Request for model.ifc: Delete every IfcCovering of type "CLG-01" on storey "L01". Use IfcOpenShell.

First a look at what the model holds.

```python
import ifcopenshell
import ifcopenshell.util.element

model = ifcopenshell.open("model.ifc")
print(model.schema)
storey = next(s for s in model.by_type("IfcBuildingStorey") if s.Name == "L01")
coverings = [e for e in ifcopenshell.util.element.get_decomposition(storey) if e.is_a("IfcCovering")]
seen = {}
for e in coverings:
    element_type = ifcopenshell.util.element.get_type(e)
    name = element_type.Name if element_type not in (None, e) else None
    seen[name] = seen.get(name, 0) + 1
for name, count in sorted(seen.items(), key=str):
    print(count, "x", name)
```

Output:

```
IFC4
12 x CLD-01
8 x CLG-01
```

```python
import ifcopenshell
import ifcopenshell.api.root
import ifcopenshell.util.element

model = ifcopenshell.open("model.ifc")

storey = next(s for s in model.by_type("IfcBuildingStorey") if s.Name == "L01")
coverings = [e for e in ifcopenshell.util.element.get_decomposition(storey) if e.is_a("IfcCovering")]
targets = [e for e in coverings if (t := ifcopenshell.util.element.get_type(e)) not in (None, e) and t.Name == "CLG-01"]

for e in targets:
    ifcopenshell.api.root.remove_product(model, product=e)
print(len(targets), "removed")

model.write("model_rev.ifc")
```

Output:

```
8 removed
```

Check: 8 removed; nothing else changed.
